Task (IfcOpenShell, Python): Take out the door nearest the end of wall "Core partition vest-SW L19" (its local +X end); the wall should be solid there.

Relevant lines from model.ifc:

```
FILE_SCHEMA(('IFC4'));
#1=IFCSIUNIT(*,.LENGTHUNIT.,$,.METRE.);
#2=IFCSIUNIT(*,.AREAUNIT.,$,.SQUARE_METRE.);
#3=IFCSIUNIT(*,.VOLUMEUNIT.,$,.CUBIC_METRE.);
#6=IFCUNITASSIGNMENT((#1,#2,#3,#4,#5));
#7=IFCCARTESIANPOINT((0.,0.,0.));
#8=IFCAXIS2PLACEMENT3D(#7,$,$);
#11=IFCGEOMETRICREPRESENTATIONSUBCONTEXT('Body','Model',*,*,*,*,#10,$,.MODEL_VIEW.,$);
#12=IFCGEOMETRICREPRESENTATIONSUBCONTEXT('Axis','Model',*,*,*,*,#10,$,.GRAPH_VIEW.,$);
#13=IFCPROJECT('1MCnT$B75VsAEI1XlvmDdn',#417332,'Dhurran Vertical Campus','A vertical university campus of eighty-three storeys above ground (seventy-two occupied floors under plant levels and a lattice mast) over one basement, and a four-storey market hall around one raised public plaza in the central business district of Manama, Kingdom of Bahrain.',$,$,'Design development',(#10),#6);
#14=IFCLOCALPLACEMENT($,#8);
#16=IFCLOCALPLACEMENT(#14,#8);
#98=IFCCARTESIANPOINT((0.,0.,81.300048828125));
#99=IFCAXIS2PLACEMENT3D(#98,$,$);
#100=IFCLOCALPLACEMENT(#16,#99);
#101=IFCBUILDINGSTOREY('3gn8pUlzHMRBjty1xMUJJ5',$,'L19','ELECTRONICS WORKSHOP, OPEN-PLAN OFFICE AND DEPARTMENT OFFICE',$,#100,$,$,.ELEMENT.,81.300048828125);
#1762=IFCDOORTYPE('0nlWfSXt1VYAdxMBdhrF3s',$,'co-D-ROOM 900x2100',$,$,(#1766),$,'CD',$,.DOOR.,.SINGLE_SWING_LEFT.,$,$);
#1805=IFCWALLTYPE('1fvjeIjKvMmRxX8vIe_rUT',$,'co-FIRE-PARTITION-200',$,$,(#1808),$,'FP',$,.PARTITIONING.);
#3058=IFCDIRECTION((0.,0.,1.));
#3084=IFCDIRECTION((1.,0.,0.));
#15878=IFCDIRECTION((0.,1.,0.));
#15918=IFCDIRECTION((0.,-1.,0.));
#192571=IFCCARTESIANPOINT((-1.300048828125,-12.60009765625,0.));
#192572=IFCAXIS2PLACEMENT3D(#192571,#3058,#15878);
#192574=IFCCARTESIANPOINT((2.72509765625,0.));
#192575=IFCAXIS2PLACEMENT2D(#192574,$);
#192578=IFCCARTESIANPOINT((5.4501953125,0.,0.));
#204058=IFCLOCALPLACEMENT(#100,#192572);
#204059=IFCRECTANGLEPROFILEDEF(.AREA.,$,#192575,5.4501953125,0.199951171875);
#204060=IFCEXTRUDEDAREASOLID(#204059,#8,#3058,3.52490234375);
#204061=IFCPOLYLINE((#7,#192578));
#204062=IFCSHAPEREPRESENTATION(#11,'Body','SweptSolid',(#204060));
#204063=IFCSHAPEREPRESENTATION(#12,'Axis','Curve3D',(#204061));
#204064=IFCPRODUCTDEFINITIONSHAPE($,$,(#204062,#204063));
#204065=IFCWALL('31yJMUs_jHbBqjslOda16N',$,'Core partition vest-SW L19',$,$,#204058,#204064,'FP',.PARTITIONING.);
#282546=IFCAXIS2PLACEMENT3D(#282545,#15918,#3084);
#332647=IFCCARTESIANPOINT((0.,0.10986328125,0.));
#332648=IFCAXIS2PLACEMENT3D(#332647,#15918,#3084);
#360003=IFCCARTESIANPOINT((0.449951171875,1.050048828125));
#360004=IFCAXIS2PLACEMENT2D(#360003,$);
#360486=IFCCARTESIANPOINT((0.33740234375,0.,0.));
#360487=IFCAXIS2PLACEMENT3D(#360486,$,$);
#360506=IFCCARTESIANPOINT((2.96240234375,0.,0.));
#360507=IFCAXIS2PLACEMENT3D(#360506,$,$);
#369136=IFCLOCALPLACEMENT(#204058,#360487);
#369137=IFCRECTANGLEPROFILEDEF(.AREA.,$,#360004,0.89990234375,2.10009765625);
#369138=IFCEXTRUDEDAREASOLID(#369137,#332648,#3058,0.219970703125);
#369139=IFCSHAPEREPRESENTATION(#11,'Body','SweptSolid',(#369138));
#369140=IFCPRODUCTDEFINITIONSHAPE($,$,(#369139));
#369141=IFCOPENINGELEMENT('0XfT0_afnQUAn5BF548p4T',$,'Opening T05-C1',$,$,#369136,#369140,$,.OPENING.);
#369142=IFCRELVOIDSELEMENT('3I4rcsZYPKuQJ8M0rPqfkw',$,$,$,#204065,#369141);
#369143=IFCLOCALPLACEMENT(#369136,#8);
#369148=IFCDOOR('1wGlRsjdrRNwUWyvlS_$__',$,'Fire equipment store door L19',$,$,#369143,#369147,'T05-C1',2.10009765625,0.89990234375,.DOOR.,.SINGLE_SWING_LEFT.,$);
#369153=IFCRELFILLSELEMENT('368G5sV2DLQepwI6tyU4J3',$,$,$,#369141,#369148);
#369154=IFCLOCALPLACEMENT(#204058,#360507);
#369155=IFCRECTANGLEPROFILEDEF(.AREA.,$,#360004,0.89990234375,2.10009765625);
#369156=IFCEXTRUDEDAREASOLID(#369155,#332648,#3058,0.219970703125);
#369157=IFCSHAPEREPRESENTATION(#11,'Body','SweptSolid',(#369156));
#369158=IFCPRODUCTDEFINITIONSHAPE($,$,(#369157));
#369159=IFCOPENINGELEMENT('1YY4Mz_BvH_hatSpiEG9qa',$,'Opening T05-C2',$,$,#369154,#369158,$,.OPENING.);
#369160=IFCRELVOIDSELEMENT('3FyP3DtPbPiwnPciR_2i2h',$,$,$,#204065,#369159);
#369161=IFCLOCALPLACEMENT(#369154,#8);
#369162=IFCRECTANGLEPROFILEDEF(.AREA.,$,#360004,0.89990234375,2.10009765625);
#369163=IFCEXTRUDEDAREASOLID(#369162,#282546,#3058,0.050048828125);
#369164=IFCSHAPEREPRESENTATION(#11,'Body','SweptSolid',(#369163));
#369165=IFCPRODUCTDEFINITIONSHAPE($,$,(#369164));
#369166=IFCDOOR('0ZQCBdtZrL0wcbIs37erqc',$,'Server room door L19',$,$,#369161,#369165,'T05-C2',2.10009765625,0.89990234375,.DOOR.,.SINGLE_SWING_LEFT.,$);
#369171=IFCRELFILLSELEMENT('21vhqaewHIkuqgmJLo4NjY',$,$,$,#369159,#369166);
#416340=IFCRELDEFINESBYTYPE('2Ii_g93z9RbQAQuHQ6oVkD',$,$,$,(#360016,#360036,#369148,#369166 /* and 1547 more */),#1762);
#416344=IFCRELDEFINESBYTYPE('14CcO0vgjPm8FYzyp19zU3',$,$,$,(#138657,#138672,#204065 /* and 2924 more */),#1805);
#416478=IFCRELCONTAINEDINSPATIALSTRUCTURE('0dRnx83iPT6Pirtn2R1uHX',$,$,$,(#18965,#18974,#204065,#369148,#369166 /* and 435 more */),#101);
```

```python
import ifcopenshell
import ifcopenshell.api.feature
import ifcopenshell.api.root
import ifcopenshell.geom
import ifcopenshell.util.shape

model = ifcopenshell.open("model.ifc")
settings = ifcopenshell.geom.settings()


def volume(element):
    """Net volume in cubic metres, openings subtracted."""
    shape = ifcopenshell.geom.create_shape(settings, element)
    return ifcopenshell.util.shape.get_volume(shape.geometry)


door = model.by_id(369166)
opening = door.FillsVoids[0].RelatingOpeningElement
wall = opening.VoidsElements[0].RelatingBuildingElement
before = volume(wall)

ifcopenshell.api.root.remove_product(model, product=door)
ifcopenshell.api.feature.remove_feature(model, feature=opening)

after = volume(wall)

print(f"wall volume {before:.3f} -> {after:.3f} m3")

model.write("model_rev.ifc")
```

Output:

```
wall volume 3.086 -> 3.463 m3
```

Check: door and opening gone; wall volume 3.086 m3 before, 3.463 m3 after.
